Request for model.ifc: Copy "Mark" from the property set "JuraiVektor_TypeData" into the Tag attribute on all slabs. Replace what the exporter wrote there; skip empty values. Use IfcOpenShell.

First a look at what the model holds.

```python
import ifcopenshell
import ifcopenshell.util.element

model = ifcopenshell.open("model.ifc")
print(model.schema)
slabs = model.by_type("IfcSlab")
print(len(slabs), "slabs")
for e in slabs[:8]:
    source = ifcopenshell.util.element.get_pset(e, "JuraiVektor_TypeData", "Mark")
    target = e.Tag
    print(e.id(), repr(source), repr(target), sep=" | ")
```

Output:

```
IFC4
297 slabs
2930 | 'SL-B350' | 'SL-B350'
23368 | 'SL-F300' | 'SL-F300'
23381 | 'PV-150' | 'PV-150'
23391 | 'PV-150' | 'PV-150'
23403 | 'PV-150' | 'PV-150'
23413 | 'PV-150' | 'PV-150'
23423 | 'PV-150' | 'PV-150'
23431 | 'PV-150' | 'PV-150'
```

```python
import ifcopenshell
import ifcopenshell.util.element

model = ifcopenshell.open("model.ifc")

count = 0
for e in model.by_type("IfcSlab"):
    value = ifcopenshell.util.element.get_pset(e, "JuraiVektor_TypeData", "Mark")
    current = e.Tag
    if not value or not value.strip() or current == value:
        continue
    e.Tag = value
    count += 1

print(count, "slabs updated")

model.write("model_updated.ifc")
```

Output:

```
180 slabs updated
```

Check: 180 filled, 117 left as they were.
